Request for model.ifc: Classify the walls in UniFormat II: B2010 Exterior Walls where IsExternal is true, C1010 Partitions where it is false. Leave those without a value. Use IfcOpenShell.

First a look at what the model holds.

```python
import ifcopenshell
import ifcopenshell.util.element

model = ifcopenshell.open("model.ifc")
print(model.schema)
print("classifications:", [c.Name for c in model.by_type("IfcClassification")])
values = [ifcopenshell.util.element.get_pset(e, "Pset_WallCommon", "IsExternal") for e in model.by_type("IfcWall")]
for value in (True, False, None):
    print("IsExternal", value, values.count(value))
```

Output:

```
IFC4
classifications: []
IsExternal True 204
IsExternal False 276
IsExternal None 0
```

```python
import ifcopenshell
import ifcopenshell.api.classification
import ifcopenshell.util.element

model = ifcopenshell.open("model.ifc")

system = ifcopenshell.api.classification.add_classification(model, classification="UniFormat II")

walls = model.by_type("IfcWall")
external = {e: ifcopenshell.util.element.get_pset(e, "Pset_WallCommon", "IsExternal") for e in walls}
for flag, code, name in ((True, "B2010", "Exterior Walls"), (False, "C1010", "Partitions")):
    products = [e for e in walls if external[e] is flag]
    ifcopenshell.api.classification.add_reference(
        model, products=products, classification=system, identification=code, name=name
    )
    print(code, len(products))

model.write("model-out.ifc")
```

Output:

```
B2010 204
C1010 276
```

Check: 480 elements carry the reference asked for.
